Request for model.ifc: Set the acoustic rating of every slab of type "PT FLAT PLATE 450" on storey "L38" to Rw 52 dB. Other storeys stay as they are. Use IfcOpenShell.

First a look at what the model holds.

```python
import ifcopenshell
import ifcopenshell.util.element

model = ifcopenshell.open("model.ifc")
print(model.schema)
storey = next(s for s in model.by_type("IfcBuildingStorey") if s.Name == "L38")
slabs = [e for e in ifcopenshell.util.element.get_decomposition(storey) if e.is_a("IfcSlab")]
seen = {}
for e in slabs:
    element_type = ifcopenshell.util.element.get_type(e)
    key = (element_type.Name if element_type != e and element_type else None, ifcopenshell.util.element.get_pset(e, "Pset_SlabCommon", "AcousticRating"))
    seen[key] = seen.get(key, 0) + 1
for (name, value), count in sorted(seen.items(), key=str):
    print(count, "x", name, "|", value)
```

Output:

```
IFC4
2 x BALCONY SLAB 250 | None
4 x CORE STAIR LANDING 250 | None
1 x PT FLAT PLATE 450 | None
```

```python
import ifcopenshell
import ifcopenshell.api.pset
import ifcopenshell.util.element

model = ifcopenshell.open("model.ifc")

storey = next(s for s in model.by_type("IfcBuildingStorey") if s.Name == "L38")
slabs = [e for e in ifcopenshell.util.element.get_decomposition(storey) if e.is_a("IfcSlab")]

count = 0
for e in slabs:
    element_type = ifcopenshell.util.element.get_type(e)
    if element_type in (None, e) or element_type.Name != "PT FLAT PLATE 450":
        continue
    found = ifcopenshell.util.element.get_pset(e, "Pset_SlabCommon", should_inherit=False)
    if found:
        pset = model.by_id(found["id"])
        if len(ifcopenshell.util.element.get_elements_by_pset(pset)) > 1:
            pset = ifcopenshell.api.pset.unshare_pset(model, products=[e], pset=pset)[0]
    else:
        pset = ifcopenshell.api.pset.add_pset(model, product=e, name="Pset_SlabCommon")
    ifcopenshell.api.pset.edit_pset(model, pset=pset, properties={"AcousticRating": "Rw 52 dB"})
    count += 1

print(count, "slabs updated")

model.write("model_rev.ifc")
```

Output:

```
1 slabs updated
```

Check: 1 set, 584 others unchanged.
